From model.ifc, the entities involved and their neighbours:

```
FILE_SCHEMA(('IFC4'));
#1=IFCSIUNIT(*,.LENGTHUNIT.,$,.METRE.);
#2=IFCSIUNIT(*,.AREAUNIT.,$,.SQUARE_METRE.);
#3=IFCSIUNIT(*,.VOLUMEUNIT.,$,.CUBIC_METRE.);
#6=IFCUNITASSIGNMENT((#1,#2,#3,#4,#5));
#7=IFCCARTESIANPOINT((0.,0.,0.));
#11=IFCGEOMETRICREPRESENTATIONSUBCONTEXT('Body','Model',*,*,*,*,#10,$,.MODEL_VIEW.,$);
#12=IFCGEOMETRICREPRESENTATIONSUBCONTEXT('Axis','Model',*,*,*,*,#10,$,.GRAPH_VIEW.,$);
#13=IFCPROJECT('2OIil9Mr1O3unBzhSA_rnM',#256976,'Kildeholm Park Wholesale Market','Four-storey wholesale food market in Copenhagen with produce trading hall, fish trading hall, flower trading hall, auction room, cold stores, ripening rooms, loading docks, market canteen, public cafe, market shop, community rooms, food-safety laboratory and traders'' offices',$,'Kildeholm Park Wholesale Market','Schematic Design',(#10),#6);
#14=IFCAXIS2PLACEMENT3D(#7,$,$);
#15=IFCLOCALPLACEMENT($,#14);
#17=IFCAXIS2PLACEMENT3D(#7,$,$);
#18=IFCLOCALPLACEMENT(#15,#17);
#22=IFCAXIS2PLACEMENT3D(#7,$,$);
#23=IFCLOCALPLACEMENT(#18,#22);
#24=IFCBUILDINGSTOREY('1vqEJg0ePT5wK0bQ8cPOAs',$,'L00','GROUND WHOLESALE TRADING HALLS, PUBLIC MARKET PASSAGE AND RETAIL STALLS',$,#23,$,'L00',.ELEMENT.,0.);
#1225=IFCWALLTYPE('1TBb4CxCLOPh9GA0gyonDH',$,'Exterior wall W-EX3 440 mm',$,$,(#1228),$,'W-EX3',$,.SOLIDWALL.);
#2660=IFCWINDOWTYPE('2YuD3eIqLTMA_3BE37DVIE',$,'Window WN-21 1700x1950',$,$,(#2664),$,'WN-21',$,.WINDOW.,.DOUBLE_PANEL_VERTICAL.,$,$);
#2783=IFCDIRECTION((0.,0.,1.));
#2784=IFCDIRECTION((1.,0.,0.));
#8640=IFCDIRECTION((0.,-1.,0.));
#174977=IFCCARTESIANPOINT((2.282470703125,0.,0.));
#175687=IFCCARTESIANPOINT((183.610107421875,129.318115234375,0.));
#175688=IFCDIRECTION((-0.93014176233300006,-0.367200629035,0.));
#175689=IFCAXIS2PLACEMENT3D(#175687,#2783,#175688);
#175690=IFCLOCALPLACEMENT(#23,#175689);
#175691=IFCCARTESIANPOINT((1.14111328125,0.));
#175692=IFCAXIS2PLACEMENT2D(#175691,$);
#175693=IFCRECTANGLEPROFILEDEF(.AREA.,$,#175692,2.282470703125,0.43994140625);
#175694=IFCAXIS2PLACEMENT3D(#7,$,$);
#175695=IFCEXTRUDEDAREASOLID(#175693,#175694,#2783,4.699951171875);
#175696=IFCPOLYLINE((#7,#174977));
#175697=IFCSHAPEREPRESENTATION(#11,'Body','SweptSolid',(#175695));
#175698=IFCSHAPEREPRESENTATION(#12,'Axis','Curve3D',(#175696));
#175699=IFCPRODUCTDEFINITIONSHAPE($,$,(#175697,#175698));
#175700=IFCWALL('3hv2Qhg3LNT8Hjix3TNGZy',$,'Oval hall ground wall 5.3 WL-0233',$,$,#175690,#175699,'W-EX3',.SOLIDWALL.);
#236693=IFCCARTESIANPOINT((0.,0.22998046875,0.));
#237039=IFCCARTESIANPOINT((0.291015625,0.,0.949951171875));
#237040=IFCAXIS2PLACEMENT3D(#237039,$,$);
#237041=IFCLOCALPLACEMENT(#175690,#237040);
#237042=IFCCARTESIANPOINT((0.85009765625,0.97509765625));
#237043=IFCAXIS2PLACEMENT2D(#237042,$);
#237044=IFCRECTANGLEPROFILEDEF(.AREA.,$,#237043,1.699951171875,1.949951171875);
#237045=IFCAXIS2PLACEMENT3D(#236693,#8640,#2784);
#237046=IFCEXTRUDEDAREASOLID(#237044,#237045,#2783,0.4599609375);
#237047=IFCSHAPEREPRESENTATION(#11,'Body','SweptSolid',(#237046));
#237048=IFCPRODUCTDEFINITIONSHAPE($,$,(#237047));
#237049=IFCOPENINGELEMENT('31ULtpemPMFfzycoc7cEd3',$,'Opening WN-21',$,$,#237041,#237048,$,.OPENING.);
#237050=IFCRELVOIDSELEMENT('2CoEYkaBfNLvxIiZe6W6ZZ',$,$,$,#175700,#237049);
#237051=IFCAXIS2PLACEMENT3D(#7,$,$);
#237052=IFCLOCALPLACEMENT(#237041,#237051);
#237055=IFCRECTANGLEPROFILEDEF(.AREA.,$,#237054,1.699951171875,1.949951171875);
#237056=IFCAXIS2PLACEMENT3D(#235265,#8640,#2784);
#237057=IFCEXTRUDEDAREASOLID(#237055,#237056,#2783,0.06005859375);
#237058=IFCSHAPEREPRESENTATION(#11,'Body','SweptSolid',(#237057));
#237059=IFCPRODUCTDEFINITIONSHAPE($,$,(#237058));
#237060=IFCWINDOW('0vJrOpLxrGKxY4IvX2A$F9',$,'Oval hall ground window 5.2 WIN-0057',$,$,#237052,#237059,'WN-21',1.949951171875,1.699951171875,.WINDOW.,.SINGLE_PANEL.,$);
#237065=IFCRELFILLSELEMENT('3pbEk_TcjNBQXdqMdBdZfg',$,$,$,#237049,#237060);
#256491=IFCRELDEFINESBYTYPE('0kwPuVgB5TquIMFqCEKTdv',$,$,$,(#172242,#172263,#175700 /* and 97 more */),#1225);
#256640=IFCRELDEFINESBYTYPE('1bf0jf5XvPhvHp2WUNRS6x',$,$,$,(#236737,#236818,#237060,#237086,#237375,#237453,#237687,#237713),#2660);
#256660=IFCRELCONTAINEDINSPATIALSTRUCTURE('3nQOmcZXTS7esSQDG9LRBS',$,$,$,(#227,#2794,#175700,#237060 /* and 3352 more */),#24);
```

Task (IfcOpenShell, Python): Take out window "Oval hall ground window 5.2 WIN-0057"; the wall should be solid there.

```python
import ifcopenshell
import ifcopenshell.api.feature
import ifcopenshell.api.root
import ifcopenshell.geom
import ifcopenshell.util.shape

model = ifcopenshell.open("model.ifc")
settings = ifcopenshell.geom.settings()


def volume(element):
    """Net volume in cubic metres, openings subtracted."""
    shape = ifcopenshell.geom.create_shape(settings, element)
    return ifcopenshell.util.shape.get_volume(shape.geometry)


window = model.by_guid("0vJrOpLxrGKxY4IvX2A$F9")
opening = window.FillsVoids[0].RelatingOpeningElement
wall = opening.VoidsElements[0].RelatingBuildingElement
before = volume(wall)

ifcopenshell.api.root.remove_product(model, product=window)
ifcopenshell.api.feature.remove_feature(model, feature=opening)

after = volume(wall)

print(f"wall volume {before:.3f} -> {after:.3f} m3")

model.write("model_edited.ifc")
```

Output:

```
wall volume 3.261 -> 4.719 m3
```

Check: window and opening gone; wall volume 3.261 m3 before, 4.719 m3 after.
